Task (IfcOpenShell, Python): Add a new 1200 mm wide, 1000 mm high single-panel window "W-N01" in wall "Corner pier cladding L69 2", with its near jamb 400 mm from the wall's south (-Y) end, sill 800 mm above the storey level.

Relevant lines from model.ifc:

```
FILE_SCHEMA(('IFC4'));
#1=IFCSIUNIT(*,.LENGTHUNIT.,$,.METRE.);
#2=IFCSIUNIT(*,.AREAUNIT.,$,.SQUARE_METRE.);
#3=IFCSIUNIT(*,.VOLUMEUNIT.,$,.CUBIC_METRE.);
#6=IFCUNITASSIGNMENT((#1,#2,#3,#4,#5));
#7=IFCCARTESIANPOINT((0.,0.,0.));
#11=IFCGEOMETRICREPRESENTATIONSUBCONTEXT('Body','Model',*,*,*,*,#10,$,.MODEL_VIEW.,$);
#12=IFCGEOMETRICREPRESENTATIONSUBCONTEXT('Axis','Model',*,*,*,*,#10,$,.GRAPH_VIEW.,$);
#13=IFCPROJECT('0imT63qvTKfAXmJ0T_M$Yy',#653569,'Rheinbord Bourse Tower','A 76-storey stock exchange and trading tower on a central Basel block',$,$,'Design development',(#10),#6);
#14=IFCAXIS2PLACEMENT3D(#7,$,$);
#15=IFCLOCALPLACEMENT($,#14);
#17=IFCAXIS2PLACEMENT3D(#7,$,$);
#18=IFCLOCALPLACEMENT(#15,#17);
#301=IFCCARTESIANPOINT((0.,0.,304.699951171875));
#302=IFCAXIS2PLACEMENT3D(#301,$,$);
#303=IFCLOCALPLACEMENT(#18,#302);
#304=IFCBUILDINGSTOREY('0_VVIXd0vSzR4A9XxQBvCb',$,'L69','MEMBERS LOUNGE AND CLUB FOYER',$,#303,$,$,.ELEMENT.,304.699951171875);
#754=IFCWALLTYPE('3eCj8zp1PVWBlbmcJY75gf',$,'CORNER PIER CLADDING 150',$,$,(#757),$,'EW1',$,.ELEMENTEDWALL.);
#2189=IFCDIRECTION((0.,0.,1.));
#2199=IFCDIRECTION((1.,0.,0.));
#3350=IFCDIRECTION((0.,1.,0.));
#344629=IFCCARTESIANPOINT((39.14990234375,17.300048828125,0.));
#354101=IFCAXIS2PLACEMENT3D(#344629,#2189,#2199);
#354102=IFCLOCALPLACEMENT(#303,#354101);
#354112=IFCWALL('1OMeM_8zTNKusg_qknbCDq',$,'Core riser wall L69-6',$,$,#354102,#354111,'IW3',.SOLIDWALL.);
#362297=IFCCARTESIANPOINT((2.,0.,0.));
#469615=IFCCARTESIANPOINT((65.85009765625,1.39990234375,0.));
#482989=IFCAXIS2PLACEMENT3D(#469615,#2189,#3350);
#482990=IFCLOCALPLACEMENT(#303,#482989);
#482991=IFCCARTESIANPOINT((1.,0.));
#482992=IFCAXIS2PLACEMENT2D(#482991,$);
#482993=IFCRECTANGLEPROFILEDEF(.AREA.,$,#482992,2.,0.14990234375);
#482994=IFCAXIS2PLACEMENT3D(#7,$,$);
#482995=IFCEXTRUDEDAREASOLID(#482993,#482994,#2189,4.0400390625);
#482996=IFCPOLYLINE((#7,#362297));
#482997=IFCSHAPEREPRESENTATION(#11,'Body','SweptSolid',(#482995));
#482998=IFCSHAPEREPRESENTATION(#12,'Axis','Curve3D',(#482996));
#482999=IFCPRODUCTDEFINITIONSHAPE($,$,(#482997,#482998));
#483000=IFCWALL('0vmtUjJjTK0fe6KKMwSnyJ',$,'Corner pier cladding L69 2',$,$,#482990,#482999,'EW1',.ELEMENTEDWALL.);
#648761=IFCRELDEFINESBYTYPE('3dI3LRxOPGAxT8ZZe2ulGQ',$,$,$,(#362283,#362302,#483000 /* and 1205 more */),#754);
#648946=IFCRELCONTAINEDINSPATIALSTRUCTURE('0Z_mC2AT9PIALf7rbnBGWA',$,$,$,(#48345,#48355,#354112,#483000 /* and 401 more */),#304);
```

```python
import numpy as np
import ifcopenshell
import ifcopenshell.api.feature
import ifcopenshell.api.geometry
import ifcopenshell.api.root
import ifcopenshell.api.spatial
import ifcopenshell.geom
import ifcopenshell.util.element
import ifcopenshell.util.placement
import ifcopenshell.util.representation
import ifcopenshell.util.shape
import ifcopenshell.util.unit

model = ifcopenshell.open("model.ifc")
unit_scale = ifcopenshell.util.unit.calculate_unit_scale(model)
settings = ifcopenshell.geom.settings()


def volume(element):
    """Net volume in cubic metres, openings subtracted."""
    shape = ifcopenshell.geom.create_shape(settings, element)
    return ifcopenshell.util.shape.get_volume(shape.geometry)


wall = model.by_guid("0vmtUjJjTK0fe6KKMwSnyJ")
storey = ifcopenshell.util.element.get_container(wall, ifc_class="IfcBuildingStorey")
context = ifcopenshell.util.representation.get_context(model, "Model", "Body", "MODEL_VIEW")
before = volume(wall)

width, height, from_end, sill = 1.2, 1, 0.4, 0.8  # metres

# The wall runs along its own X axis, and the end named is its -X end.
wall_shape = ifcopenshell.geom.create_shape(settings, wall)
x, y, z = ifcopenshell.util.shape.get_vertices(wall_shape.geometry).T
start = x.min() + from_end
face, thickness = float(y.min()), float(y.max() - y.min())
wall_matrix = ifcopenshell.util.placement.get_local_placement(wall.ObjectPlacement)
level = ifcopenshell.util.placement.get_local_placement(storey.ObjectPlacement)[2, 3]


def in_wall(x, y):
    """Placement at x, y metres in the wall's axes, at sill height."""
    matrix = wall_matrix.copy()
    matrix[:, 3] = wall_matrix @ np.array([x / unit_scale, y / unit_scale, 0.0, 1.0])
    matrix[2, 3] = level + sill / unit_scale
    return matrix


# Opening: a box that overshoots both wall faces by 50 mm.
opening = ifcopenshell.api.root.create_entity(model, ifc_class="IfcOpeningElement", predefined_type="OPENING")
box = ifcopenshell.api.geometry.add_wall_representation(
    model, context=context, length=width, height=height, thickness=thickness + 0.1
)
ifcopenshell.api.geometry.assign_representation(model, product=opening, representation=box)
ifcopenshell.api.geometry.edit_object_placement(model, product=opening, matrix=in_wall(start, face - 0.05), is_si=False)
ifcopenshell.api.feature.add_feature(model, feature=opening, element=wall)

window = ifcopenshell.api.root.create_entity(model, ifc_class="IfcWindow", name="W-N01", predefined_type="WINDOW")
window.OverallWidth, window.OverallHeight = width / unit_scale, height / unit_scale
window.PartitioningType = "SINGLE_PANEL"
body = ifcopenshell.api.geometry.add_window_representation(
    model,
    context=context,
    overall_width=window.OverallWidth,
    overall_height=window.OverallHeight,
    partition_type="SINGLE_PANEL",
)
ifcopenshell.api.geometry.assign_representation(model, product=window, representation=body)
ifcopenshell.api.spatial.assign_container(model, products=[window], relating_structure=storey)
ifcopenshell.api.feature.add_filling(model, opening=opening, element=window)

# Centre the window in the wall's thickness.
ifcopenshell.api.geometry.edit_object_placement(model, product=window, matrix=in_wall(start, face), is_si=False)
window_shape = ifcopenshell.geom.create_shape(settings, window)
depth = ifcopenshell.util.shape.get_vertices(window_shape.geometry)[:, 1]
offset = face + thickness / 2 - (depth.min() + depth.max()) / 2
ifcopenshell.api.geometry.edit_object_placement(model, product=window, matrix=in_wall(start, offset), is_si=False)

after = volume(wall)

print(f"wall volume {before:.3f} -> {after:.3f} m3")

model.write("model_rev.ifc")
```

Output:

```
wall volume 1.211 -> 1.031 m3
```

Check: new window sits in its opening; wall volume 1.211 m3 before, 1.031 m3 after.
